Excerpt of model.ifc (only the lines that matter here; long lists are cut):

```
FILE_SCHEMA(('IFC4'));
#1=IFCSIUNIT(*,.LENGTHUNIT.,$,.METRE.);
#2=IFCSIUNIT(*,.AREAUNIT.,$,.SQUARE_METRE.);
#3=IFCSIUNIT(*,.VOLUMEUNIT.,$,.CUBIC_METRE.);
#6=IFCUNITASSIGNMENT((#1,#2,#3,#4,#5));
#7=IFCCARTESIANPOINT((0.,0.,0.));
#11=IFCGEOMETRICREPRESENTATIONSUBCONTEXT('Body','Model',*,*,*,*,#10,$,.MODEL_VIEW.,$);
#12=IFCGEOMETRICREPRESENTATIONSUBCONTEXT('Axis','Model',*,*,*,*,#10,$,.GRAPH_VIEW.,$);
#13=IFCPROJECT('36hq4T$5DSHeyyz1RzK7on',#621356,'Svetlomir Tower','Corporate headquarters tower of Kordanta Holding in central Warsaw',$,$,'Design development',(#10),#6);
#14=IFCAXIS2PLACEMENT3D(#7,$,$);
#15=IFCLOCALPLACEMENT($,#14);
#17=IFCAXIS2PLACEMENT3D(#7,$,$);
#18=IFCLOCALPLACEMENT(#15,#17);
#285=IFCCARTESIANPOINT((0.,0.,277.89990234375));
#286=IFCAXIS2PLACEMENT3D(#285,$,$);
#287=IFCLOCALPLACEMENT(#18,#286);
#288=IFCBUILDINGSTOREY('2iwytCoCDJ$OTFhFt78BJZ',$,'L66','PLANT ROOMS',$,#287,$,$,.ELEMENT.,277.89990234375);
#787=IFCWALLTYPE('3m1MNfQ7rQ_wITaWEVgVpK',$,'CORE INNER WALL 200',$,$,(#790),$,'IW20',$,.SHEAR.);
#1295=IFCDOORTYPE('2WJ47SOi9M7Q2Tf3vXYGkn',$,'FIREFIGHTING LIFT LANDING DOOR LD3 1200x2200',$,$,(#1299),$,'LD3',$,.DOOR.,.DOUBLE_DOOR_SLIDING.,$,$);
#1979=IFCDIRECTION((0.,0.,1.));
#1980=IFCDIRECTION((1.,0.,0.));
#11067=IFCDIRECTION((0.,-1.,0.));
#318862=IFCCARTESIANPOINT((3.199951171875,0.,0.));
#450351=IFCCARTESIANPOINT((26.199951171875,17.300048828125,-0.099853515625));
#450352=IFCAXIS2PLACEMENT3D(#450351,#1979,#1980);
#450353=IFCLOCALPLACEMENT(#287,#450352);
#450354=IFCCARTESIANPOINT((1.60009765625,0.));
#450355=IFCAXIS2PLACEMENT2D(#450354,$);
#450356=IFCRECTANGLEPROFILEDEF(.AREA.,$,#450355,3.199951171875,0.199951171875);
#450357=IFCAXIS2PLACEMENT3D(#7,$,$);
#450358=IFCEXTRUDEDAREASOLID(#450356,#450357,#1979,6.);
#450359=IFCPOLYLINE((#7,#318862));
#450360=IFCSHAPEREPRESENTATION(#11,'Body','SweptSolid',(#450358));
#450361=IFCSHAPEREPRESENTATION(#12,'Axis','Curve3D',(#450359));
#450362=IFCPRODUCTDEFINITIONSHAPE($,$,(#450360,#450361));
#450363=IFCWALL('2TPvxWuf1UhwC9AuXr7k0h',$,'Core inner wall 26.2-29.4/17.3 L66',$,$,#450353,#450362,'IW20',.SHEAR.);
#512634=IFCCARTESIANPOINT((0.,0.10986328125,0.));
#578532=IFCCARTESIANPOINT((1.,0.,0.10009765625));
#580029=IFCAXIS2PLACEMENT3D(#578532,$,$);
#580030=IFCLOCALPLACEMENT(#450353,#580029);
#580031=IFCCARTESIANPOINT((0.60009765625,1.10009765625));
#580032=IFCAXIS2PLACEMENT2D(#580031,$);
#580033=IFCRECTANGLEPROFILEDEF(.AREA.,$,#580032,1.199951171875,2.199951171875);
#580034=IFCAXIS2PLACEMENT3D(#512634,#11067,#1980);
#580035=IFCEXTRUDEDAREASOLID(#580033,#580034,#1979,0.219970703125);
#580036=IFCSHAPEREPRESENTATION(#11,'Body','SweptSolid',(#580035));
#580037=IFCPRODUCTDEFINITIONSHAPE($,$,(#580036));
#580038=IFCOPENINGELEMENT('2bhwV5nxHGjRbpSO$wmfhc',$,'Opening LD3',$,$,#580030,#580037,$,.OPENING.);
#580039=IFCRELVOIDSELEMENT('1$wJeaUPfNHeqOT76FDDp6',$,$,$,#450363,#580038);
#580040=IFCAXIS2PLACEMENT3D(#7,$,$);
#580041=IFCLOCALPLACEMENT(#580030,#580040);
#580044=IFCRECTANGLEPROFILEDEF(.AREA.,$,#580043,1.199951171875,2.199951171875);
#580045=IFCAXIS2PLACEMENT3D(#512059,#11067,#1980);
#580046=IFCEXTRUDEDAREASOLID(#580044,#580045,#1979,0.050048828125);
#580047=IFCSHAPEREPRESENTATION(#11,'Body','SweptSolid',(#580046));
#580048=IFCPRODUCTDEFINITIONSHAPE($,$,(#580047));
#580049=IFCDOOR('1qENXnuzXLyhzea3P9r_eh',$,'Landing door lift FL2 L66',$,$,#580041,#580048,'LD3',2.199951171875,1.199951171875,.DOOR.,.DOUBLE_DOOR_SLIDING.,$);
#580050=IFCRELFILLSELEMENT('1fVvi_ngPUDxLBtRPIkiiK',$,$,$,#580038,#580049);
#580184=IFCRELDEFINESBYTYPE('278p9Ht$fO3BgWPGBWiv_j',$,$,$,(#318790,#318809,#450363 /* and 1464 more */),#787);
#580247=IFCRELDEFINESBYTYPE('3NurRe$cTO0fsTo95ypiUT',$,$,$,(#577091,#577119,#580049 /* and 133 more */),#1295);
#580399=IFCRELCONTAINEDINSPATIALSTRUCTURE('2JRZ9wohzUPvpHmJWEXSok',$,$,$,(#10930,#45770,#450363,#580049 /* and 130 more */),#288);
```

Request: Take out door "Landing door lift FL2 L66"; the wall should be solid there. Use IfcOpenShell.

```python
import ifcopenshell
import ifcopenshell.api.feature
import ifcopenshell.api.root
import ifcopenshell.geom
import ifcopenshell.util.shape

model = ifcopenshell.open("model.ifc")
settings = ifcopenshell.geom.settings()


def volume(element):
    """Net volume in cubic metres, openings subtracted."""
    shape = ifcopenshell.geom.create_shape(settings, element)
    return ifcopenshell.util.shape.get_volume(shape.geometry)


door = model.by_guid("1qENXnuzXLyhzea3P9r_eh")
opening = door.FillsVoids[0].RelatingOpeningElement
wall = opening.VoidsElements[0].RelatingBuildingElement
before = volume(wall)

ifcopenshell.api.root.remove_product(model, product=door)
ifcopenshell.api.feature.remove_feature(model, feature=opening)

after = volume(wall)

print(f"wall volume {before:.3f} -> {after:.3f} m3")

model.write("model_updated.ifc")
```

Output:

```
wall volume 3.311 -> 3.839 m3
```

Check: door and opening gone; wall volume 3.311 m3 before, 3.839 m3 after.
